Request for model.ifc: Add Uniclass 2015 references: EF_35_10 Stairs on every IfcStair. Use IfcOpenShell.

First a look at what the model holds.

```python
import ifcopenshell

model = ifcopenshell.open("model.ifc")
print(model.schema)
print("classifications:", [c.Name for c in model.by_type("IfcClassification")])
for ifc_class in ("IfcDoor", "IfcRoof", "IfcStair", "IfcWall", "IfcWindow"):
    print(ifc_class, len(model.by_type(ifc_class)))
```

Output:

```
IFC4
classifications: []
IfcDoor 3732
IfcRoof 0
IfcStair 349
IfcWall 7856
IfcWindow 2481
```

```python
import ifcopenshell
import ifcopenshell.api.classification

model = ifcopenshell.open("model.ifc")

system = ifcopenshell.api.classification.add_classification(model, classification="Uniclass 2015")

codes = {
    "IfcStair": ("EF_35_10", "Stairs"),
}
for ifc_class, (code, name) in codes.items():
    products = model.by_type(ifc_class)
    ifcopenshell.api.classification.add_reference(
        model, products=products, classification=system, identification=code, name=name
    )
    print(code, len(products))

model.write("model_v2.ifc")
```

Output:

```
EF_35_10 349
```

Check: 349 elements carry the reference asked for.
